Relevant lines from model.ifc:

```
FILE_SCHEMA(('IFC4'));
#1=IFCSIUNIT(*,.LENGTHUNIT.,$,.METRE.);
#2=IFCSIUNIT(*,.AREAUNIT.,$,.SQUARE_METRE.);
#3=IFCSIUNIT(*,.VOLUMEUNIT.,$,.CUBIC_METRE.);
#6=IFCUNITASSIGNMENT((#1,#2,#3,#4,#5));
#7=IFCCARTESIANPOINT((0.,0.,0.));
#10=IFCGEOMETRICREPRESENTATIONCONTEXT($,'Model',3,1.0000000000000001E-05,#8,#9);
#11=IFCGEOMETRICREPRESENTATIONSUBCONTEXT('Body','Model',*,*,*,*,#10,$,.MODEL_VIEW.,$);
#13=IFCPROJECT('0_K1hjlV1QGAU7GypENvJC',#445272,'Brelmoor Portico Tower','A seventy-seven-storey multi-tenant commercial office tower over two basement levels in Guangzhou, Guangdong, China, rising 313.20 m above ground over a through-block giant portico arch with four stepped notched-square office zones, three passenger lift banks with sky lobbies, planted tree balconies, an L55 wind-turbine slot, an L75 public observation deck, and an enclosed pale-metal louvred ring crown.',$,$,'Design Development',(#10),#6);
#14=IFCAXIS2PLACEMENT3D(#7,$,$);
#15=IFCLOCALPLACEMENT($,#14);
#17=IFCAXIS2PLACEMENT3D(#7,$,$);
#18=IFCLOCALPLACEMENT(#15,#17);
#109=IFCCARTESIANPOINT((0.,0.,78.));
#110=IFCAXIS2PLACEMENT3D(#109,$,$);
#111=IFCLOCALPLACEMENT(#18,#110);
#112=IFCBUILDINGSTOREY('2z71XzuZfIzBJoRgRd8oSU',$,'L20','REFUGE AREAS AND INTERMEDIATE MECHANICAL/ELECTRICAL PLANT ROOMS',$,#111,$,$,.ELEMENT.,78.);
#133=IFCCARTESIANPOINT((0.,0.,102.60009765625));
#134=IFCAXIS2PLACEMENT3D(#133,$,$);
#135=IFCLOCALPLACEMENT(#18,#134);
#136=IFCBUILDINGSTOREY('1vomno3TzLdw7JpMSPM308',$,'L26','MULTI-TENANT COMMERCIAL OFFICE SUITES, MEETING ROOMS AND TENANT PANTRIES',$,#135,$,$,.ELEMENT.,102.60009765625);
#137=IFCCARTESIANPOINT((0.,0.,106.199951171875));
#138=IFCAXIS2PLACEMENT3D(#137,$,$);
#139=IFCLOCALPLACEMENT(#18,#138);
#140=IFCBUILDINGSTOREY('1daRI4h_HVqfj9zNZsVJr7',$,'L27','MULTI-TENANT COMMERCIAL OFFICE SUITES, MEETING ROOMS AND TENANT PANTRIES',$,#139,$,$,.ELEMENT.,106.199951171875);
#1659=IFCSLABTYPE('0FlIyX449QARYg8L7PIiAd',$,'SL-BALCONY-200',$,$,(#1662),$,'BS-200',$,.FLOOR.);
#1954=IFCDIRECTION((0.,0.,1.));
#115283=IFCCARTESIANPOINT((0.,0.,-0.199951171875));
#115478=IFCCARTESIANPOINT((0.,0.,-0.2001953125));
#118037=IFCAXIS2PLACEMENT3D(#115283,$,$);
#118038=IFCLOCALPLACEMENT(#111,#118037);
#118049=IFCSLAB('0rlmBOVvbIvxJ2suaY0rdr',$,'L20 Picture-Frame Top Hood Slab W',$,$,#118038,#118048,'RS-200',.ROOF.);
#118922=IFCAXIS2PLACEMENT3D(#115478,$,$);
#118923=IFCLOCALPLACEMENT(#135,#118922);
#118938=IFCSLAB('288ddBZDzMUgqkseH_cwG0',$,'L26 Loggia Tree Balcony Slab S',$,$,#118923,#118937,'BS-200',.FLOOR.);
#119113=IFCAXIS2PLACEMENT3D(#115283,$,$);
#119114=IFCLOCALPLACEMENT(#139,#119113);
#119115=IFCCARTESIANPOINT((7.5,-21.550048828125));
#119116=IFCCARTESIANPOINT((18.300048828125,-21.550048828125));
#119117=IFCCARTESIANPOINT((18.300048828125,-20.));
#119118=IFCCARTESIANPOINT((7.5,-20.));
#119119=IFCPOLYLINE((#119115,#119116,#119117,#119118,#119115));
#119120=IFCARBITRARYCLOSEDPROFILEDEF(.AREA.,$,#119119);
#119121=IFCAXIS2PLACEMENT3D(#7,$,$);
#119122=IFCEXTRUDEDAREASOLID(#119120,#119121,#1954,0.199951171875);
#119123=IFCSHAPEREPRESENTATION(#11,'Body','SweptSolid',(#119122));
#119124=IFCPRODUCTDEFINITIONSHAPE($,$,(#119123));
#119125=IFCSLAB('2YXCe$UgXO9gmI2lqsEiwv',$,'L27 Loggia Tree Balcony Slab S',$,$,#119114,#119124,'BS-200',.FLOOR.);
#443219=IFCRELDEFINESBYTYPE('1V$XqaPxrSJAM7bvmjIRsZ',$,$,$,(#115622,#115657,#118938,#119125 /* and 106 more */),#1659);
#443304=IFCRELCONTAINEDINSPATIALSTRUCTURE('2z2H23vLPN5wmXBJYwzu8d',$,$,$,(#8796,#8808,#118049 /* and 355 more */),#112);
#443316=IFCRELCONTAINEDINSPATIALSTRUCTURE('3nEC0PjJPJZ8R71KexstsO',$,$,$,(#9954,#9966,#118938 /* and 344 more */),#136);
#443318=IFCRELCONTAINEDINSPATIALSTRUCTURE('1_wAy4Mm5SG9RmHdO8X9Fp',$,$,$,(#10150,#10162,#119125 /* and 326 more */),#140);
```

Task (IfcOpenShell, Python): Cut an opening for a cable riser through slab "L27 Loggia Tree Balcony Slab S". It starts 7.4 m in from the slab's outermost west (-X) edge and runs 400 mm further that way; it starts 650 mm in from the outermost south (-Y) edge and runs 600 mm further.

```python
import numpy as np
import ifcopenshell
import ifcopenshell.api.feature
import ifcopenshell.api.geometry
import ifcopenshell.api.root
import ifcopenshell.geom
import ifcopenshell.util.placement
import ifcopenshell.util.representation
import ifcopenshell.util.shape
import ifcopenshell.util.unit

model = ifcopenshell.open("model.ifc")
unit_scale = ifcopenshell.util.unit.calculate_unit_scale(model)
settings = ifcopenshell.geom.settings()


def volume(element):
    """Net volume in cubic metres, openings subtracted."""
    shape = ifcopenshell.geom.create_shape(settings, element)
    return ifcopenshell.util.shape.get_volume(shape.geometry)


slab = model.by_guid("2YXCe$UgXO9gmI2lqsEiwv")
before = volume(slab)

# Extent in the slab's own axes, in metres. The edges named are its -X and -Y sides.
slab_shape = ifcopenshell.geom.create_shape(settings, slab)
vertices = ifcopenshell.util.shape.get_vertices(slab_shape.geometry)
x_min, y_min, bottom = vertices.min(axis=0)
top = vertices[:, 2].max()

opening = ifcopenshell.api.root.create_entity(model, ifc_class="IfcOpeningElement", name="Cable riser opening", predefined_type="OPENING")
context = ifcopenshell.util.representation.get_context(model, "Model", "Body", "MODEL_VIEW")
width, depth = 0.4, 0.6
outline = [(0.0, 0.0), (width, 0.0), (width, depth), (0.0, depth), (0.0, 0.0)]
# Overshoot both faces by 50 mm so the cut is clean.
shape = ifcopenshell.api.geometry.add_slab_representation(
    model, context=context, depth=top - bottom + 0.1, polyline=outline
)
ifcopenshell.api.geometry.assign_representation(model, product=opening, representation=shape)

matrix = ifcopenshell.util.placement.get_local_placement(slab.ObjectPlacement)
matrix[:, 3] = matrix @ np.append(np.array([x_min + 7.4, y_min + 0.65, bottom - 0.05]) / unit_scale, 1.0)
ifcopenshell.api.geometry.edit_object_placement(model, product=opening, matrix=matrix, is_si=False)
ifcopenshell.api.feature.add_feature(model, feature=opening, element=slab)

after = volume(slab)

print(f"slab volume {before:.3f} -> {after:.3f} m3")

model.write("model_v2.ifc")
```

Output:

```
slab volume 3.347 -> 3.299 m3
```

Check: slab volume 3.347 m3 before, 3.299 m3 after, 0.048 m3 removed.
